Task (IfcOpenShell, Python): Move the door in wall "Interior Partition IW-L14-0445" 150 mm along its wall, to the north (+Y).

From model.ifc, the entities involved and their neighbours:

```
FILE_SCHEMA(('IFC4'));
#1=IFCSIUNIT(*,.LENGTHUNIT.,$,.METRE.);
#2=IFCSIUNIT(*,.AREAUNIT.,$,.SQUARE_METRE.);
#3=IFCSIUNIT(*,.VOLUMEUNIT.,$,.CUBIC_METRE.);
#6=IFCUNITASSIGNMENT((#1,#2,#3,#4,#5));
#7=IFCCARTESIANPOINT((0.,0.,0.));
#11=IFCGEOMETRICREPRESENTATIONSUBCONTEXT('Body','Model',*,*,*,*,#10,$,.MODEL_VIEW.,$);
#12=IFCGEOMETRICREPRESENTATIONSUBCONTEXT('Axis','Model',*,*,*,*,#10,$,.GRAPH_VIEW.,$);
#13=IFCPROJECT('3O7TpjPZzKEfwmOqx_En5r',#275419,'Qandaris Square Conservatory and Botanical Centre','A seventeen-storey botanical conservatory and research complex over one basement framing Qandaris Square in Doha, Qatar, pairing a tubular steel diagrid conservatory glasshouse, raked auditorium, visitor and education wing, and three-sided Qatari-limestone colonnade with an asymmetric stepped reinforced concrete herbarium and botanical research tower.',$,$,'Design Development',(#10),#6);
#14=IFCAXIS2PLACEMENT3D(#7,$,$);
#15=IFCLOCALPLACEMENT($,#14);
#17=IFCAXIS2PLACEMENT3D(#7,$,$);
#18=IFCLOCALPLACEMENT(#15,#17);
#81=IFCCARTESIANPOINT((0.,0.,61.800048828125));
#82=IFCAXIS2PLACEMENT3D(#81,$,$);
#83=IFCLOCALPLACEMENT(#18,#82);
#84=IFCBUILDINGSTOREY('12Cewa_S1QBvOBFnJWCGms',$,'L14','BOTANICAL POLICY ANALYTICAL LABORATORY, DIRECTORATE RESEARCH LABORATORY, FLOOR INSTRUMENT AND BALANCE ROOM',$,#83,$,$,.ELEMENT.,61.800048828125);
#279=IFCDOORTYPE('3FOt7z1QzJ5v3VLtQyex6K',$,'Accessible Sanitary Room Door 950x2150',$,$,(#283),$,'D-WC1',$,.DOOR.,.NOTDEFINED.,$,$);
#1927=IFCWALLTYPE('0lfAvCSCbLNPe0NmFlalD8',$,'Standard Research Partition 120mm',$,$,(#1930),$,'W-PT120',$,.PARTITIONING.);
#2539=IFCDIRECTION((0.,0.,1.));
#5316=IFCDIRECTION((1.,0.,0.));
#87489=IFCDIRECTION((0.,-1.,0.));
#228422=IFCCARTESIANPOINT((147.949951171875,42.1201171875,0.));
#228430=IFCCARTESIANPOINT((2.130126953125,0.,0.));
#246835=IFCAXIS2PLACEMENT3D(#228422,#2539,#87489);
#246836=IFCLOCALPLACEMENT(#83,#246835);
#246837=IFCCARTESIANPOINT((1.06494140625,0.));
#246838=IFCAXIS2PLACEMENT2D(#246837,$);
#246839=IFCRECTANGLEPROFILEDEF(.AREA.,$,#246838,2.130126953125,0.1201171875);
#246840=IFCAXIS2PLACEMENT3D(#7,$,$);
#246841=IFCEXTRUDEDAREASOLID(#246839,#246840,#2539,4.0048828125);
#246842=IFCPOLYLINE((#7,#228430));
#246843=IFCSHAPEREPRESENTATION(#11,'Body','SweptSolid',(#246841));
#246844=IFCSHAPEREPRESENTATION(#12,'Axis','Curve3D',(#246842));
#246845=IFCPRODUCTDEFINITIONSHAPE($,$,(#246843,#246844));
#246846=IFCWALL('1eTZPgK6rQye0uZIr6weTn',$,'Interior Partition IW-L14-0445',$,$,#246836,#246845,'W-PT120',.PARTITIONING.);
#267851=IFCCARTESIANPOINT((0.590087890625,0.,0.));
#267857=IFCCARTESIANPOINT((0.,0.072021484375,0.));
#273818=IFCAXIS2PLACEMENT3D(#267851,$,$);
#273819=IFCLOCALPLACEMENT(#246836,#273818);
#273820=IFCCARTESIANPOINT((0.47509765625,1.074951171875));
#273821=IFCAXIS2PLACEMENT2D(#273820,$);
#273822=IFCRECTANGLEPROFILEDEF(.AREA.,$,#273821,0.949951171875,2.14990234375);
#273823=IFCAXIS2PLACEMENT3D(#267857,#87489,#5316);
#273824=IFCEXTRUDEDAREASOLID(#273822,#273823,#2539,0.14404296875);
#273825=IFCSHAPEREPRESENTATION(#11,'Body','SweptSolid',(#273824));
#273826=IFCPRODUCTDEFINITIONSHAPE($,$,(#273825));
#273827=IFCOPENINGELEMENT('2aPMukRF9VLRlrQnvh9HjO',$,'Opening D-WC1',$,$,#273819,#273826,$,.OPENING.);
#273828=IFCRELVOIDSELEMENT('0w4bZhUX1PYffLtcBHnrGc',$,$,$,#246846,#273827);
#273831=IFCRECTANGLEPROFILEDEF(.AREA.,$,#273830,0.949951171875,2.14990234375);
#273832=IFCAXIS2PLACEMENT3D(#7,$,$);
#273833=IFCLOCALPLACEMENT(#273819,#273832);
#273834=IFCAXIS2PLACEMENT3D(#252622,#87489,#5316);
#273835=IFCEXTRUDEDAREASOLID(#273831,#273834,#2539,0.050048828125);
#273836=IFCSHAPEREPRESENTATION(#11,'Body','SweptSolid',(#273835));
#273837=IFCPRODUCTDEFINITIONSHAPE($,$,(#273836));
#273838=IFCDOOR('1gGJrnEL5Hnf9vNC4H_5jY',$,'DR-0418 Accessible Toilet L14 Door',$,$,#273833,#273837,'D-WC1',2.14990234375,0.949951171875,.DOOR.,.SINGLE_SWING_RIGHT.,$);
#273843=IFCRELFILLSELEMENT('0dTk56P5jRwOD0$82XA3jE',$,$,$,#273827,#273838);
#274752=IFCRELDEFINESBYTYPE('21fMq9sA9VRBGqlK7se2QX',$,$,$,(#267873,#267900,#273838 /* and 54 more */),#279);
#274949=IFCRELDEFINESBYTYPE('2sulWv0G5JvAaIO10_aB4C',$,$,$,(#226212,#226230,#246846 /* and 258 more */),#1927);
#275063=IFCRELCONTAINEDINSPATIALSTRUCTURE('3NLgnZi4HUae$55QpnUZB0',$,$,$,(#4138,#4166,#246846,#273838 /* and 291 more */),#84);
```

```python
import ifcopenshell
import ifcopenshell.api.geometry
import ifcopenshell.util.placement
import ifcopenshell.util.unit

model = ifcopenshell.open("model.ifc")
unit_scale = ifcopenshell.util.unit.calculate_unit_scale(model)

door = model.by_guid("1gGJrnEL5Hnf9vNC4H_5jY")
opening = door.FillsVoids[0].RelatingOpeningElement
wall = opening.VoidsElements[0].RelatingBuildingElement

wall_matrix = ifcopenshell.util.placement.get_local_placement(wall.ObjectPlacement)
shift = wall_matrix[:3, 0] * -0.15 / unit_scale
before = ifcopenshell.util.placement.get_local_placement(door.ObjectPlacement)[:3, 3].copy()

# The door is placed relative to its opening, so it follows when the opening moves.
matrix = ifcopenshell.util.placement.get_local_placement(opening.ObjectPlacement)
matrix[:3, 3] += shift
ifcopenshell.api.geometry.edit_object_placement(
    model, product=opening, matrix=matrix, is_si=False, should_transform_children=True
)

after = ifcopenshell.util.placement.get_local_placement(door.ObjectPlacement)[:3, 3]
print("door moved by", (after - before).round(3) + 0.0)

model.write("model_edited.ifc")
```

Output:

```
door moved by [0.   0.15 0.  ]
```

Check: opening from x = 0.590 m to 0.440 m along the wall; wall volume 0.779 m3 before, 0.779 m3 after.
